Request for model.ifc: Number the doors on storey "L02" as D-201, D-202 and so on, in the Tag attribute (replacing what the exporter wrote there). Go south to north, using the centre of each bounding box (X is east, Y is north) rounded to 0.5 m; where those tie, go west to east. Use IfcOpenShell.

First a look at what the model holds.

```python
import ifcopenshell
import ifcopenshell.util.element
import ifcopenshell.util.placement

model = ifcopenshell.open("model.ifc")
print(model.schema)
storey = next(s for s in model.by_type("IfcBuildingStorey") if s.Name == "L02")
doors = [e for e in ifcopenshell.util.element.get_decomposition(storey) if e.is_a("IfcDoor")]
for e in sorted(doors, key=lambda e: e.id()):
    origin = ifcopenshell.util.placement.get_local_placement(e.ObjectPlacement)[:3, 3]
    print(e.id(), e.Tag, e.Name, origin.round(2) + 0.0, sep=" | ")
```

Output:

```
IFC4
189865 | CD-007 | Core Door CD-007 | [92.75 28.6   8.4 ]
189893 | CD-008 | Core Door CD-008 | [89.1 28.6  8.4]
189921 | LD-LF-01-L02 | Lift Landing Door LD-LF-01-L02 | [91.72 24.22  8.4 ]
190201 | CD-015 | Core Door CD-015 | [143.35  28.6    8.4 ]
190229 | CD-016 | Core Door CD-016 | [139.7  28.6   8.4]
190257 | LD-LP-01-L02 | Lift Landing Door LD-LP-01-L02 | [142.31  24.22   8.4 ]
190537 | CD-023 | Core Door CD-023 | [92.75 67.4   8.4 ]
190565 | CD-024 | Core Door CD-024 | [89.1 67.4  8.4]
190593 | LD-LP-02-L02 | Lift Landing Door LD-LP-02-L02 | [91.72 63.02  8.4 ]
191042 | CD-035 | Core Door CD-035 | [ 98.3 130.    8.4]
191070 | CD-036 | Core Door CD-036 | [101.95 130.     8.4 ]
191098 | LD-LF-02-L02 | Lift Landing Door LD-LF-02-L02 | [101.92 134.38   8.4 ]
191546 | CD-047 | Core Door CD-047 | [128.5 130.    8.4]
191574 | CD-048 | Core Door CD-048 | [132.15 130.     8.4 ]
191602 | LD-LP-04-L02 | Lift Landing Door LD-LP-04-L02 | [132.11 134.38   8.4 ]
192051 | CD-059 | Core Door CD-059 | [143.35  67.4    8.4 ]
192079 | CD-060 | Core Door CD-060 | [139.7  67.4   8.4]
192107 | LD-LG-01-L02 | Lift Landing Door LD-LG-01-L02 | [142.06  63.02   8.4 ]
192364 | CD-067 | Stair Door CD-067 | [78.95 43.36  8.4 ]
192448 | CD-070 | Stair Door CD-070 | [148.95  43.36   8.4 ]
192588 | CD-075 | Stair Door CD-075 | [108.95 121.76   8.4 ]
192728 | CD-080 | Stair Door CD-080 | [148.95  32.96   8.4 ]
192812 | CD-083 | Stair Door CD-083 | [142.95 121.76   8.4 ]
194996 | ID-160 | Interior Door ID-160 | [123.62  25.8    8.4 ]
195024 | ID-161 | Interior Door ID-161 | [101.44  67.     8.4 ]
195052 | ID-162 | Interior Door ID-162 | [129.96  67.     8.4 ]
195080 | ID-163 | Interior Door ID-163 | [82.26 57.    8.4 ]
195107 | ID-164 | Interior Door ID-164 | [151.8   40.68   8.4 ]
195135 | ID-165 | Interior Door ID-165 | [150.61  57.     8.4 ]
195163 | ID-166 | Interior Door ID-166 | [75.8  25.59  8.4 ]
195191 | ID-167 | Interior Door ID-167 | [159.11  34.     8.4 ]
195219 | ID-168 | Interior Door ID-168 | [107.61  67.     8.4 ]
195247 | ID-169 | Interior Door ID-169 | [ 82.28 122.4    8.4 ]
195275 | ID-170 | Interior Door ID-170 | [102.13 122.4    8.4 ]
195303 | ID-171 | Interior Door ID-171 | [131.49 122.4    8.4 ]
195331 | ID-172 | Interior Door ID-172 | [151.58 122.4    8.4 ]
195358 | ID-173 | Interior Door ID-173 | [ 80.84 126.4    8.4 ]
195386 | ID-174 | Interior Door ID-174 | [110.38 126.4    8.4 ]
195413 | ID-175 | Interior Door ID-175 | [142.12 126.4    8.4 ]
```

```python
import ifcopenshell
import ifcopenshell.geom
import ifcopenshell.util.element
import ifcopenshell.util.shape

model = ifcopenshell.open("model.ifc")
settings = ifcopenshell.geom.settings()
settings.set("use-world-coords", True)


def centre(element):
    shape = ifcopenshell.geom.create_shape(settings, element)
    return ifcopenshell.util.shape.get_bbox_centroid(shape.geometry)


storey = next(s for s in model.by_type("IfcBuildingStorey") if s.Name == "L02")
doors = [e for e in ifcopenshell.util.element.get_decomposition(storey) if e.is_a("IfcDoor")]

# Insertion points can sit at a corner or the storey origin, so sort by the geometry (in metres).
centres = {e: centre(e) for e in doors}
doors.sort(key=lambda e: (round(centres[e][1] / 0.5), centres[e][0]))

for i, e in enumerate(doors, start=1):
    number = f"D-2{i:02d}"
    e.Tag = number
    print(e.id(), number)

model.write("model_edited.ifc")
```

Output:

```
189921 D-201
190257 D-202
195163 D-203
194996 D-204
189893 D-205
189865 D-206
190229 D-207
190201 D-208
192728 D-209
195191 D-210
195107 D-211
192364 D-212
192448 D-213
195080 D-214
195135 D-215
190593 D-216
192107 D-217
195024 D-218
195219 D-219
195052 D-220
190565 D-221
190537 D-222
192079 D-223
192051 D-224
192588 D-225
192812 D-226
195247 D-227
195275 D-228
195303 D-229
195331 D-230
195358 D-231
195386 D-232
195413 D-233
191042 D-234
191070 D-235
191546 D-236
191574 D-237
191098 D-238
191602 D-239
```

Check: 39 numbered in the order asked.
